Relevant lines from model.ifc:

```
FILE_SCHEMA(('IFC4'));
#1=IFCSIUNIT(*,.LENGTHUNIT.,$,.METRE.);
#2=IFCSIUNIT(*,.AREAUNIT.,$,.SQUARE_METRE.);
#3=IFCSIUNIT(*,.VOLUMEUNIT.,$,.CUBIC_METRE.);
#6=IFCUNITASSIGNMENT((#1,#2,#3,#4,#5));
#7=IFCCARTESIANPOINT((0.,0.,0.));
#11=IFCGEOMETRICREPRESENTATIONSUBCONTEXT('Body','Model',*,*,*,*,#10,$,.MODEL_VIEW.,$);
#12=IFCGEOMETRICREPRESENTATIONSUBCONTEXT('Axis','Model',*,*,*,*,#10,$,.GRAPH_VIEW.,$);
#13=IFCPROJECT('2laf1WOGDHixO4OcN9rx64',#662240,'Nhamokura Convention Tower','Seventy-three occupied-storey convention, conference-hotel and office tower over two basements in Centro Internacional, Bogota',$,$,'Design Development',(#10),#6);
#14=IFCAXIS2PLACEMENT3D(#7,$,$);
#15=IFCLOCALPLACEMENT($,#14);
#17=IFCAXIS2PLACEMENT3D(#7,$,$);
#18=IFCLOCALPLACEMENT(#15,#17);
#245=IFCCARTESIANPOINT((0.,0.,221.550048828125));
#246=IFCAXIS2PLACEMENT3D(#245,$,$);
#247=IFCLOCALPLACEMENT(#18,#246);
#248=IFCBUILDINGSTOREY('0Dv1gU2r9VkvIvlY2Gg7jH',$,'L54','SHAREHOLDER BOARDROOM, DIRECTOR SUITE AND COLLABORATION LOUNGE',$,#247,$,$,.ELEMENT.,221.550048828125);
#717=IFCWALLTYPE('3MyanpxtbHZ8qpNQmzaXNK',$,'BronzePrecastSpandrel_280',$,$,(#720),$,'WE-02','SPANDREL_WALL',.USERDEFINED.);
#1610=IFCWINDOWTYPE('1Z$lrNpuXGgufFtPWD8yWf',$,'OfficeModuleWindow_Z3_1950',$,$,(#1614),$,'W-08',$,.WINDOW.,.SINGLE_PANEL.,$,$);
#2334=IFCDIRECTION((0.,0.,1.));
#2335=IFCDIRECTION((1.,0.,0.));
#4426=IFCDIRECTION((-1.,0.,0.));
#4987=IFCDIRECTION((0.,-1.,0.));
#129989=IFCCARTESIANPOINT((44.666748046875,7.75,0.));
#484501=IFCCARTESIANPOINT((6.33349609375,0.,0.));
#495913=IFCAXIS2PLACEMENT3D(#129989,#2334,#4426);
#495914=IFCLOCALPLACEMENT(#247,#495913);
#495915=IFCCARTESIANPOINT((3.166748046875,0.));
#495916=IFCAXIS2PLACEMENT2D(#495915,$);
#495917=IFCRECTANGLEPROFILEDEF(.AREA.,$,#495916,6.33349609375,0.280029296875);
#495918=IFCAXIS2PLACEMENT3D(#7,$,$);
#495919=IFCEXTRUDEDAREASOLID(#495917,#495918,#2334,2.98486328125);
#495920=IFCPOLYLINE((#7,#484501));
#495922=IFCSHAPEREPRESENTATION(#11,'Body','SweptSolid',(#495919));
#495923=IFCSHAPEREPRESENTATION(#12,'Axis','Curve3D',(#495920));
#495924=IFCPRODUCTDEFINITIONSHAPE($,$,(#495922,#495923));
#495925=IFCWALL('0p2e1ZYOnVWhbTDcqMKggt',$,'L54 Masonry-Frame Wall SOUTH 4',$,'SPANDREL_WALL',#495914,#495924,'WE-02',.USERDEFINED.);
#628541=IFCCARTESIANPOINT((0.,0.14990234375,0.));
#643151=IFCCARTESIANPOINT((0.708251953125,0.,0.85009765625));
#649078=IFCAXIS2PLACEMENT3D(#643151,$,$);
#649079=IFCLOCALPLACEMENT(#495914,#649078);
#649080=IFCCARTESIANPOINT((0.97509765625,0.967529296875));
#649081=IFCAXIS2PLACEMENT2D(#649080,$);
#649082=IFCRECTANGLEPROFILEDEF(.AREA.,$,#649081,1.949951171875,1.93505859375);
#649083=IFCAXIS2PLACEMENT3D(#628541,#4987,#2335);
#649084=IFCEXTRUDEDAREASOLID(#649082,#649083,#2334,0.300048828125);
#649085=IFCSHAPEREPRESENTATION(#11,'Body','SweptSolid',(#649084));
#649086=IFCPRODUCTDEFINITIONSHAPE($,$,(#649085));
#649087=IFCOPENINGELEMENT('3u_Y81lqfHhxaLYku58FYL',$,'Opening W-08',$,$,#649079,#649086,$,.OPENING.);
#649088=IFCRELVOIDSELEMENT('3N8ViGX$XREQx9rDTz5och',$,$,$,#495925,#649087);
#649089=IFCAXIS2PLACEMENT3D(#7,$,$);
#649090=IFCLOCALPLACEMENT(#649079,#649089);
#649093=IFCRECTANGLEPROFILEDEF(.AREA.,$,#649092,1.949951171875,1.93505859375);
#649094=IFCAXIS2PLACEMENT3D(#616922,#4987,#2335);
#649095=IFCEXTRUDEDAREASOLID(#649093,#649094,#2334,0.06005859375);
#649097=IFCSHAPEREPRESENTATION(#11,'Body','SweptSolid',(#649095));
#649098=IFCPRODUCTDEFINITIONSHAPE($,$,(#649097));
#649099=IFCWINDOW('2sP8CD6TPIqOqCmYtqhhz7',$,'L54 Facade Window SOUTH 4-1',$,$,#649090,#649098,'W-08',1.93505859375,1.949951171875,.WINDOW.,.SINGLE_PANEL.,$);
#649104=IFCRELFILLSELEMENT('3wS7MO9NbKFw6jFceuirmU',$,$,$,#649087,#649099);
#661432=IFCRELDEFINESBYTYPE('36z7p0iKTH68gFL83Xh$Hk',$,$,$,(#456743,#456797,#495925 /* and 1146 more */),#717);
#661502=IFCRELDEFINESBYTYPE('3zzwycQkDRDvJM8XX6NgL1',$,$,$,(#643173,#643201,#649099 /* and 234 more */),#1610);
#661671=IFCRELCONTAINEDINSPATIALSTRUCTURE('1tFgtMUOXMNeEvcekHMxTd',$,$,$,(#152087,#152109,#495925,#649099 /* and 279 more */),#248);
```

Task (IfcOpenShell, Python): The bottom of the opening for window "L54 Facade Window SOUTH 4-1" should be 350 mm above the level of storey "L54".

```python
import numpy as np
import ifcopenshell
import ifcopenshell.api.geometry
import ifcopenshell.geom
import ifcopenshell.util.element
import ifcopenshell.util.placement
import ifcopenshell.util.shape
import ifcopenshell.util.unit

model = ifcopenshell.open("model.ifc")
unit_scale = ifcopenshell.util.unit.calculate_unit_scale(model)

window = model.by_guid("2sP8CD6TPIqOqCmYtqhhz7")
opening = window.FillsVoids[0].RelatingOpeningElement
storey = ifcopenshell.util.element.get_container(window, ifc_class="IfcBuildingStorey")
level = ifcopenshell.util.placement.get_local_placement(storey.ObjectPlacement)[2, 3]

# The opening's origin need not be at the sill, so measure its lowest point.
shape = ifcopenshell.geom.create_shape(ifcopenshell.geom.settings(), opening)
bottom = ifcopenshell.util.shape.get_shape_bottom_elevation(shape, shape.geometry) / unit_scale
dz = level + 0.35 / unit_scale - bottom

shift = np.array([0.0, 0.0, dz])
# The window is placed relative to its opening, so it follows when the opening moves.
matrix = ifcopenshell.util.placement.get_local_placement(opening.ObjectPlacement)
matrix[:3, 3] += shift
ifcopenshell.api.geometry.edit_object_placement(
    model, product=opening, matrix=matrix, is_si=False, should_transform_children=True
)

print(f"moved by {dz * unit_scale:+.3f} m")

model.write("model_updated.ifc")
```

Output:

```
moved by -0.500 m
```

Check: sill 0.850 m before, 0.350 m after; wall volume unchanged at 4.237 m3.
